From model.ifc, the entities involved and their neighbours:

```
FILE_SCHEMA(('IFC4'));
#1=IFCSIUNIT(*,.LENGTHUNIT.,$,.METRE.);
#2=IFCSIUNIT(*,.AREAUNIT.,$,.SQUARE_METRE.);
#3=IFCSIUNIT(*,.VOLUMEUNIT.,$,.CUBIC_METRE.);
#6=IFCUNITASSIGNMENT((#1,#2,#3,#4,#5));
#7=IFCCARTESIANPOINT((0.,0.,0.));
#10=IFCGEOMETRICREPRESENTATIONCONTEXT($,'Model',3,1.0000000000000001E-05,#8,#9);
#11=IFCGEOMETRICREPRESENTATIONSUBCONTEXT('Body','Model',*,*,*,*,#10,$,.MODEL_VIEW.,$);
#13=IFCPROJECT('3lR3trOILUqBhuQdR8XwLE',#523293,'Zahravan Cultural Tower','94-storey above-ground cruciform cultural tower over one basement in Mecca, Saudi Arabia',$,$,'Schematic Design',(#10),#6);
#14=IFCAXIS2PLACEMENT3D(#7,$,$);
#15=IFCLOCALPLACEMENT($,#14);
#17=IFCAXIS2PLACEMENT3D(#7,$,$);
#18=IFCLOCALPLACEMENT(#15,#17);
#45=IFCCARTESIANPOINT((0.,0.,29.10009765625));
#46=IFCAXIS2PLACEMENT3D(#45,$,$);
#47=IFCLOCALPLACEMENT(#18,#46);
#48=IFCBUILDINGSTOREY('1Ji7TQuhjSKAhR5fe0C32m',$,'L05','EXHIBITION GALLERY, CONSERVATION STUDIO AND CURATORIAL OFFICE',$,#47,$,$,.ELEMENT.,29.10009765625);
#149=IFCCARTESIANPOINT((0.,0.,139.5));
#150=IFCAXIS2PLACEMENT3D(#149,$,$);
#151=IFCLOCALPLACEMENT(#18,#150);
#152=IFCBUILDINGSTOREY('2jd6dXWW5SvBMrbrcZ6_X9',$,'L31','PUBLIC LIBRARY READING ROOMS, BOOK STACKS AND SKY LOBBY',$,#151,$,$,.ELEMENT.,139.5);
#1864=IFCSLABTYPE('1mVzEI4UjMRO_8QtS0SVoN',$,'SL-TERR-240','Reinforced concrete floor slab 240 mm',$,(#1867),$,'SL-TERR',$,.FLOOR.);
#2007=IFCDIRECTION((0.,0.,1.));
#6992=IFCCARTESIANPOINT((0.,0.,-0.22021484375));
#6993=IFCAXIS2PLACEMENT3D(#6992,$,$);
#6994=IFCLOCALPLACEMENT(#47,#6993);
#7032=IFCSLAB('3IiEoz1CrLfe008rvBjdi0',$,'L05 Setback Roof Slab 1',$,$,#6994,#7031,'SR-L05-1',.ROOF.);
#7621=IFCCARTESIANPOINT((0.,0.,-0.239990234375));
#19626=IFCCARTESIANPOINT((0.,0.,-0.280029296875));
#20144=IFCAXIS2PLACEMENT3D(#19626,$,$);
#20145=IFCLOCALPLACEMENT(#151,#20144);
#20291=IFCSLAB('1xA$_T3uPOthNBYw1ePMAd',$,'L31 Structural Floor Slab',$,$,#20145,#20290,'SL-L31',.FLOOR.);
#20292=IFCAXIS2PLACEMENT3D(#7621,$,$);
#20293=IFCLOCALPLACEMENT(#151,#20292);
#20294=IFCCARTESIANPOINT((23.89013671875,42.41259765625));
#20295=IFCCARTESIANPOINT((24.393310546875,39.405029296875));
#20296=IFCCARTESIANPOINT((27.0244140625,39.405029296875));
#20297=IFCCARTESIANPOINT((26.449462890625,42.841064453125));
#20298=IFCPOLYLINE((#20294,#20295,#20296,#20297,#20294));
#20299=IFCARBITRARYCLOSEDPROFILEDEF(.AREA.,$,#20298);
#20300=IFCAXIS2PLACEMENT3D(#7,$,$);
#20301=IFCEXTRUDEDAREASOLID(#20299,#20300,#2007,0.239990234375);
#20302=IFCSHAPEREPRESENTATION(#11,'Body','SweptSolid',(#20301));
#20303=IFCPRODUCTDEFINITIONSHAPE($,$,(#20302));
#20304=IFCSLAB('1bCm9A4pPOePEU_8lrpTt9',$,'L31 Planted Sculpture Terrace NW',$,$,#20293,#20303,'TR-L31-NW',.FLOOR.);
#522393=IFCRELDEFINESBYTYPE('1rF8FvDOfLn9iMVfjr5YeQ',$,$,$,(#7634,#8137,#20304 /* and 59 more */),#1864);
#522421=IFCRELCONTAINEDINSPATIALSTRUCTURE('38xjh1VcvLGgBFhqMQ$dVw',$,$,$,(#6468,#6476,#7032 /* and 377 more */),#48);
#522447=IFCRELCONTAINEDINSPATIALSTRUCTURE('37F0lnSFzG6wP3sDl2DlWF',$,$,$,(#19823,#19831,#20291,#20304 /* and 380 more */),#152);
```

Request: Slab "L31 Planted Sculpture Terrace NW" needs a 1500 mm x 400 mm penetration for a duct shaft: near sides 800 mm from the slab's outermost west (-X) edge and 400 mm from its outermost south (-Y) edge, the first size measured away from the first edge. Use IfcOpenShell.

```python
import numpy as np
import ifcopenshell
import ifcopenshell.api.feature
import ifcopenshell.api.geometry
import ifcopenshell.api.root
import ifcopenshell.geom
import ifcopenshell.util.placement
import ifcopenshell.util.representation
import ifcopenshell.util.shape
import ifcopenshell.util.unit

model = ifcopenshell.open("model.ifc")
unit_scale = ifcopenshell.util.unit.calculate_unit_scale(model)
settings = ifcopenshell.geom.settings()


def volume(element):
    """Net volume in cubic metres, openings subtracted."""
    shape = ifcopenshell.geom.create_shape(settings, element)
    return ifcopenshell.util.shape.get_volume(shape.geometry)


slab = model.by_guid("1bCm9A4pPOePEU_8lrpTt9")
before = volume(slab)

# Extent in the slab's own axes, in metres. The edges named are its -X and -Y sides.
slab_shape = ifcopenshell.geom.create_shape(settings, slab)
vertices = ifcopenshell.util.shape.get_vertices(slab_shape.geometry)
x_min, y_min, bottom = vertices.min(axis=0)
top = vertices[:, 2].max()

opening = ifcopenshell.api.root.create_entity(model, ifc_class="IfcOpeningElement", name="Duct shaft opening", predefined_type="OPENING")
context = ifcopenshell.util.representation.get_context(model, "Model", "Body", "MODEL_VIEW")
width, depth = 1.5, 0.4
outline = [(0.0, 0.0), (width, 0.0), (width, depth), (0.0, depth), (0.0, 0.0)]
# Overshoot both faces by 50 mm so the cut is clean.
shape = ifcopenshell.api.geometry.add_slab_representation(
    model, context=context, depth=top - bottom + 0.1, polyline=outline
)
ifcopenshell.api.geometry.assign_representation(model, product=opening, representation=shape)

matrix = ifcopenshell.util.placement.get_local_placement(slab.ObjectPlacement)
matrix[:, 3] = matrix @ np.append(np.array([x_min + 0.8, y_min + 0.4, bottom - 0.05]) / unit_scale, 1.0)
ifcopenshell.api.geometry.edit_object_placement(model, product=opening, matrix=matrix, is_si=False)
ifcopenshell.api.feature.add_feature(model, feature=opening, element=slab)

after = volume(slab)

print(f"slab volume {before:.3f} -> {after:.3f} m3")

model.write("model_rev.ifc")
```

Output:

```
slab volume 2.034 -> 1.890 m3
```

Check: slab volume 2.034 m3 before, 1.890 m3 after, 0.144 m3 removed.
